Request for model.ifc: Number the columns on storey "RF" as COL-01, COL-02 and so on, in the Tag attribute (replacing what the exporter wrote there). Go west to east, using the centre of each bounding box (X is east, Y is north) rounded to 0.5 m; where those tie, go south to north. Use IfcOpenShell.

First a look at what the model holds.

```python
import ifcopenshell
import ifcopenshell.util.element
import ifcopenshell.util.placement

model = ifcopenshell.open("model.ifc")
print(model.schema)
storey = next(s for s in model.by_type("IfcBuildingStorey") if s.Name == "RF")
columns = [e for e in ifcopenshell.util.element.get_decomposition(storey) if e.is_a("IfcColumn")]
for e in sorted(columns, key=lambda e: e.id()):
    origin = ifcopenshell.util.placement.get_local_placement(e.ObjectPlacement)[:3, 3]
    print(e.id(), e.Tag, e.Name, origin.round(2) + 0.0, sep=" | ")
```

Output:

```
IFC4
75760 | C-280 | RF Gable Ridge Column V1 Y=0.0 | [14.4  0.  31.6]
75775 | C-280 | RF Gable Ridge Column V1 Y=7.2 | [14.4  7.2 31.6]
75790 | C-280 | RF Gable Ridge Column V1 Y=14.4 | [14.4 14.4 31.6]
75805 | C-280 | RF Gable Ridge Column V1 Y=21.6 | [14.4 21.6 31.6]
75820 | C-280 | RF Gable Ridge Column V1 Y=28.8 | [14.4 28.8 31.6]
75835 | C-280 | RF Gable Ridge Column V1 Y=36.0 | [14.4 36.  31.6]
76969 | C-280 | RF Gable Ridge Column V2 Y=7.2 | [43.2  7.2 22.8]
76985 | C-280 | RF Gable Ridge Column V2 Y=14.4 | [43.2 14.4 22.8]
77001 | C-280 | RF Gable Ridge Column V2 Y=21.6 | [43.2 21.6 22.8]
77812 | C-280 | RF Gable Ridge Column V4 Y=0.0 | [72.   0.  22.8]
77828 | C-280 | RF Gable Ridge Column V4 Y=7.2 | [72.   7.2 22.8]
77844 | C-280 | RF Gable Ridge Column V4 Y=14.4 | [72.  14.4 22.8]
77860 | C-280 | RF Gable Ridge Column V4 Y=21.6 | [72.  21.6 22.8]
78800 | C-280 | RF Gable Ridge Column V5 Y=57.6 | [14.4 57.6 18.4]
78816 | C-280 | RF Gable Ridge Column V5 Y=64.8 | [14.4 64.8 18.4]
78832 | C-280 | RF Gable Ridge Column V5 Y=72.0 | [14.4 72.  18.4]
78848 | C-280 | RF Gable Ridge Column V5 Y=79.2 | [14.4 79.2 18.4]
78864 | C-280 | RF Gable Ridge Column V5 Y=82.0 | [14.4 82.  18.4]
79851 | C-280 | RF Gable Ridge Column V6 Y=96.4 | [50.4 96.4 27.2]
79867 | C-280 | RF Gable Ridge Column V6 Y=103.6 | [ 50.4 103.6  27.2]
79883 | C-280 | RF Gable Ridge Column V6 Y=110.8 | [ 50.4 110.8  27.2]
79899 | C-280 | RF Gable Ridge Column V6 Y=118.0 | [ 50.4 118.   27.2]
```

```python
import ifcopenshell
import ifcopenshell.geom
import ifcopenshell.util.element
import ifcopenshell.util.shape

model = ifcopenshell.open("model.ifc")
settings = ifcopenshell.geom.settings()
settings.set("use-world-coords", True)


def centre(element):
    shape = ifcopenshell.geom.create_shape(settings, element)
    return ifcopenshell.util.shape.get_bbox_centroid(shape.geometry)


storey = next(s for s in model.by_type("IfcBuildingStorey") if s.Name == "RF")
columns = [e for e in ifcopenshell.util.element.get_decomposition(storey) if e.is_a("IfcColumn")]

# Insertion points can sit at a corner or the storey origin, so sort by the geometry (in metres).
centres = {e: centre(e) for e in columns}
columns.sort(key=lambda e: (round(centres[e][0] / 0.5), centres[e][1]))

for i, e in enumerate(columns, start=1):
    number = f"COL-{i:02d}"
    e.Tag = number
    print(e.id(), number)

model.write("model_rev.ifc")
```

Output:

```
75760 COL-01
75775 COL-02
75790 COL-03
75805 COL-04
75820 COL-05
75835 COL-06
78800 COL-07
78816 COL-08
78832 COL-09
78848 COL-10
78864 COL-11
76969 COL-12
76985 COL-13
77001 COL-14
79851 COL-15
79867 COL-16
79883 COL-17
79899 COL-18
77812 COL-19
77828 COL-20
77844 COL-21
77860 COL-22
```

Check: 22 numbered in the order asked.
